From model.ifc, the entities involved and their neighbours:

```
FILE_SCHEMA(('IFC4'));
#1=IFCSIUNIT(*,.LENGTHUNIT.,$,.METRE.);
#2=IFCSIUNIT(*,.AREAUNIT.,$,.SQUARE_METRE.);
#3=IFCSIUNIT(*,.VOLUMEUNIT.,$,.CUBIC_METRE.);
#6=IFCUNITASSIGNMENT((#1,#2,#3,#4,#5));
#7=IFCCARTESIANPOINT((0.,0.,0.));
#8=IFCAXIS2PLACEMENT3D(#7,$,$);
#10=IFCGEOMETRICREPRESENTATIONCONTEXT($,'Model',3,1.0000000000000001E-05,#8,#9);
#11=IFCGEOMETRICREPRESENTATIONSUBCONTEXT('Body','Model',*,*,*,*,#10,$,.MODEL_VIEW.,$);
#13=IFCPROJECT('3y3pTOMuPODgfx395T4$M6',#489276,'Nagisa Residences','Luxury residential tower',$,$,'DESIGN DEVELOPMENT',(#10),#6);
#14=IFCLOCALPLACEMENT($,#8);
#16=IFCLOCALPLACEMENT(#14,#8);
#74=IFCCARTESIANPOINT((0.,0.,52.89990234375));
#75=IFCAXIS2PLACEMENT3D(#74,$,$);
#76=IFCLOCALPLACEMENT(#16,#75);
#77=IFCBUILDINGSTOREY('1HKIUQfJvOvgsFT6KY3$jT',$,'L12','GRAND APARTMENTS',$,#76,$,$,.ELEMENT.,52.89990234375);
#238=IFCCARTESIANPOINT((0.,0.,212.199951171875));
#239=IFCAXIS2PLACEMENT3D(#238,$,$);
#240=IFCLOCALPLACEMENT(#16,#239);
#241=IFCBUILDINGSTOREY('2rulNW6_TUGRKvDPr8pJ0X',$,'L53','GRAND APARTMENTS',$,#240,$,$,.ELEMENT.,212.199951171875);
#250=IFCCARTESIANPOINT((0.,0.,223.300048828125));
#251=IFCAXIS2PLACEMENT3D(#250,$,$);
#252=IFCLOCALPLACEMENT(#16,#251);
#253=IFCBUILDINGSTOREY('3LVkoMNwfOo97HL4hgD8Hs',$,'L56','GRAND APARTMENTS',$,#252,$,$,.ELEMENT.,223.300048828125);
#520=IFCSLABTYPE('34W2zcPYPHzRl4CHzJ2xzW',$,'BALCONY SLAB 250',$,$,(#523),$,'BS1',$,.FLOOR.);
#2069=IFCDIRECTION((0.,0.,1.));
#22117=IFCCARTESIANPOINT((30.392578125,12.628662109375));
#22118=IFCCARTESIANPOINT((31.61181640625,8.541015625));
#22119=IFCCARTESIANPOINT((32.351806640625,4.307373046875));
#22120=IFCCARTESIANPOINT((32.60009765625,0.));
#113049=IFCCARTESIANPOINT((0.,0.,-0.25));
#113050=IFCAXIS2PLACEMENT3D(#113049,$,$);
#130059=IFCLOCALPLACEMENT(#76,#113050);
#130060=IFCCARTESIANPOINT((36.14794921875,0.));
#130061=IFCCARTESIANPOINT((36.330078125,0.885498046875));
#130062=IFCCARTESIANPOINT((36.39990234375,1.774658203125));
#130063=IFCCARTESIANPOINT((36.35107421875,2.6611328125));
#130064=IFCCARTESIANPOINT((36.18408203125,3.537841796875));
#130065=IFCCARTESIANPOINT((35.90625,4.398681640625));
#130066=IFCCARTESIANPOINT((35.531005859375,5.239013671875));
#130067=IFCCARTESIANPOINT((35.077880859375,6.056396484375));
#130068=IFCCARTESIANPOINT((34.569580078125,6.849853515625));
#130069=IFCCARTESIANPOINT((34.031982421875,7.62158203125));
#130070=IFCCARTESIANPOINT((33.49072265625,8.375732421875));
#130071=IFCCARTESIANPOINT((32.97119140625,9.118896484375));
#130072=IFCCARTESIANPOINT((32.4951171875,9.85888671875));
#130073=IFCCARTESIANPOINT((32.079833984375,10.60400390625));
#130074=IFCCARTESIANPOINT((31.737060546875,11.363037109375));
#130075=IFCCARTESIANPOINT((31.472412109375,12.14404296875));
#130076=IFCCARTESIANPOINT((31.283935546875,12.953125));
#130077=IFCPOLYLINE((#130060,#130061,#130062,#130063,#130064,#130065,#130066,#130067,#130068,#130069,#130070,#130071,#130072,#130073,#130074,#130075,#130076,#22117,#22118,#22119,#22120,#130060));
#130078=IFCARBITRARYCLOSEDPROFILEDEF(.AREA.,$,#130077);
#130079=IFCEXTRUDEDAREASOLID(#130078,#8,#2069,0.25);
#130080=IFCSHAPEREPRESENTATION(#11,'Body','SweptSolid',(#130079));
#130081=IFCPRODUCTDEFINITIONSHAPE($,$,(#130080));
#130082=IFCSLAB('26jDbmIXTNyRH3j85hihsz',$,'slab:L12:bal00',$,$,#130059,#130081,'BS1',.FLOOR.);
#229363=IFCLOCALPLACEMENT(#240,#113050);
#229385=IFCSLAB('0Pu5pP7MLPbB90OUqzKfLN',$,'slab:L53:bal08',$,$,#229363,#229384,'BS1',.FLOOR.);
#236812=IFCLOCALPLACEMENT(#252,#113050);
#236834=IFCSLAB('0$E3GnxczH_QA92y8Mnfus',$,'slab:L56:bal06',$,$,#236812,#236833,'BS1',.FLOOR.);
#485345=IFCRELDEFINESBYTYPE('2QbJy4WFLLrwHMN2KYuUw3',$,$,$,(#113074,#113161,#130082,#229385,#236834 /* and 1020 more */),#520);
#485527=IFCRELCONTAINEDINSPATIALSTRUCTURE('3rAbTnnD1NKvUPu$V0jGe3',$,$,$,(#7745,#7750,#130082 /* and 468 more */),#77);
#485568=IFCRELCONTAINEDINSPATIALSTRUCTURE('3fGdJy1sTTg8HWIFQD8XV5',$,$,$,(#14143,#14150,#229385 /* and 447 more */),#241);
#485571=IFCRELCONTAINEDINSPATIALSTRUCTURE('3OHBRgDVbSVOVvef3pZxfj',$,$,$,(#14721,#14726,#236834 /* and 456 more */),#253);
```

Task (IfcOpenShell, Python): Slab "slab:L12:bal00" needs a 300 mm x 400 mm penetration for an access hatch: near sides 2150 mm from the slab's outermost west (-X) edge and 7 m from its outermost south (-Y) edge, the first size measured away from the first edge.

```python
import numpy as np
import ifcopenshell
import ifcopenshell.api.feature
import ifcopenshell.api.geometry
import ifcopenshell.api.root
import ifcopenshell.geom
import ifcopenshell.util.placement
import ifcopenshell.util.representation
import ifcopenshell.util.shape
import ifcopenshell.util.unit

model = ifcopenshell.open("model.ifc")
unit_scale = ifcopenshell.util.unit.calculate_unit_scale(model)
settings = ifcopenshell.geom.settings()


def volume(element):
    """Net volume in cubic metres, openings subtracted."""
    shape = ifcopenshell.geom.create_shape(settings, element)
    return ifcopenshell.util.shape.get_volume(shape.geometry)


slab = model.by_guid("26jDbmIXTNyRH3j85hihsz")
before = volume(slab)

# Extent in the slab's own axes, in metres. The edges named are its -X and -Y sides.
slab_shape = ifcopenshell.geom.create_shape(settings, slab)
vertices = ifcopenshell.util.shape.get_vertices(slab_shape.geometry)
x_min, y_min, bottom = vertices.min(axis=0)
top = vertices[:, 2].max()

opening = ifcopenshell.api.root.create_entity(model, ifc_class="IfcOpeningElement", name="Access hatch opening", predefined_type="OPENING")
context = ifcopenshell.util.representation.get_context(model, "Model", "Body", "MODEL_VIEW")
width, depth = 0.3, 0.4
outline = [(0.0, 0.0), (width, 0.0), (width, depth), (0.0, depth), (0.0, 0.0)]
# Overshoot both faces by 50 mm so the cut is clean.
shape = ifcopenshell.api.geometry.add_slab_representation(
    model, context=context, depth=top - bottom + 0.1, polyline=outline
)
ifcopenshell.api.geometry.assign_representation(model, product=opening, representation=shape)

matrix = ifcopenshell.util.placement.get_local_placement(slab.ObjectPlacement)
matrix[:, 3] = matrix @ np.append(np.array([x_min + 2.15, y_min + 7, bottom - 0.05]) / unit_scale, 1.0)
ifcopenshell.api.geometry.edit_object_placement(model, product=opening, matrix=matrix, is_si=False)
ifcopenshell.api.feature.add_feature(model, feature=opening, element=slab)

after = volume(slab)

print(f"slab volume {before:.3f} -> {after:.3f} m3")

model.write("model_v2.ifc")
```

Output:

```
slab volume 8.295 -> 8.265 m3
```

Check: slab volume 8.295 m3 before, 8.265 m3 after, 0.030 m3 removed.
